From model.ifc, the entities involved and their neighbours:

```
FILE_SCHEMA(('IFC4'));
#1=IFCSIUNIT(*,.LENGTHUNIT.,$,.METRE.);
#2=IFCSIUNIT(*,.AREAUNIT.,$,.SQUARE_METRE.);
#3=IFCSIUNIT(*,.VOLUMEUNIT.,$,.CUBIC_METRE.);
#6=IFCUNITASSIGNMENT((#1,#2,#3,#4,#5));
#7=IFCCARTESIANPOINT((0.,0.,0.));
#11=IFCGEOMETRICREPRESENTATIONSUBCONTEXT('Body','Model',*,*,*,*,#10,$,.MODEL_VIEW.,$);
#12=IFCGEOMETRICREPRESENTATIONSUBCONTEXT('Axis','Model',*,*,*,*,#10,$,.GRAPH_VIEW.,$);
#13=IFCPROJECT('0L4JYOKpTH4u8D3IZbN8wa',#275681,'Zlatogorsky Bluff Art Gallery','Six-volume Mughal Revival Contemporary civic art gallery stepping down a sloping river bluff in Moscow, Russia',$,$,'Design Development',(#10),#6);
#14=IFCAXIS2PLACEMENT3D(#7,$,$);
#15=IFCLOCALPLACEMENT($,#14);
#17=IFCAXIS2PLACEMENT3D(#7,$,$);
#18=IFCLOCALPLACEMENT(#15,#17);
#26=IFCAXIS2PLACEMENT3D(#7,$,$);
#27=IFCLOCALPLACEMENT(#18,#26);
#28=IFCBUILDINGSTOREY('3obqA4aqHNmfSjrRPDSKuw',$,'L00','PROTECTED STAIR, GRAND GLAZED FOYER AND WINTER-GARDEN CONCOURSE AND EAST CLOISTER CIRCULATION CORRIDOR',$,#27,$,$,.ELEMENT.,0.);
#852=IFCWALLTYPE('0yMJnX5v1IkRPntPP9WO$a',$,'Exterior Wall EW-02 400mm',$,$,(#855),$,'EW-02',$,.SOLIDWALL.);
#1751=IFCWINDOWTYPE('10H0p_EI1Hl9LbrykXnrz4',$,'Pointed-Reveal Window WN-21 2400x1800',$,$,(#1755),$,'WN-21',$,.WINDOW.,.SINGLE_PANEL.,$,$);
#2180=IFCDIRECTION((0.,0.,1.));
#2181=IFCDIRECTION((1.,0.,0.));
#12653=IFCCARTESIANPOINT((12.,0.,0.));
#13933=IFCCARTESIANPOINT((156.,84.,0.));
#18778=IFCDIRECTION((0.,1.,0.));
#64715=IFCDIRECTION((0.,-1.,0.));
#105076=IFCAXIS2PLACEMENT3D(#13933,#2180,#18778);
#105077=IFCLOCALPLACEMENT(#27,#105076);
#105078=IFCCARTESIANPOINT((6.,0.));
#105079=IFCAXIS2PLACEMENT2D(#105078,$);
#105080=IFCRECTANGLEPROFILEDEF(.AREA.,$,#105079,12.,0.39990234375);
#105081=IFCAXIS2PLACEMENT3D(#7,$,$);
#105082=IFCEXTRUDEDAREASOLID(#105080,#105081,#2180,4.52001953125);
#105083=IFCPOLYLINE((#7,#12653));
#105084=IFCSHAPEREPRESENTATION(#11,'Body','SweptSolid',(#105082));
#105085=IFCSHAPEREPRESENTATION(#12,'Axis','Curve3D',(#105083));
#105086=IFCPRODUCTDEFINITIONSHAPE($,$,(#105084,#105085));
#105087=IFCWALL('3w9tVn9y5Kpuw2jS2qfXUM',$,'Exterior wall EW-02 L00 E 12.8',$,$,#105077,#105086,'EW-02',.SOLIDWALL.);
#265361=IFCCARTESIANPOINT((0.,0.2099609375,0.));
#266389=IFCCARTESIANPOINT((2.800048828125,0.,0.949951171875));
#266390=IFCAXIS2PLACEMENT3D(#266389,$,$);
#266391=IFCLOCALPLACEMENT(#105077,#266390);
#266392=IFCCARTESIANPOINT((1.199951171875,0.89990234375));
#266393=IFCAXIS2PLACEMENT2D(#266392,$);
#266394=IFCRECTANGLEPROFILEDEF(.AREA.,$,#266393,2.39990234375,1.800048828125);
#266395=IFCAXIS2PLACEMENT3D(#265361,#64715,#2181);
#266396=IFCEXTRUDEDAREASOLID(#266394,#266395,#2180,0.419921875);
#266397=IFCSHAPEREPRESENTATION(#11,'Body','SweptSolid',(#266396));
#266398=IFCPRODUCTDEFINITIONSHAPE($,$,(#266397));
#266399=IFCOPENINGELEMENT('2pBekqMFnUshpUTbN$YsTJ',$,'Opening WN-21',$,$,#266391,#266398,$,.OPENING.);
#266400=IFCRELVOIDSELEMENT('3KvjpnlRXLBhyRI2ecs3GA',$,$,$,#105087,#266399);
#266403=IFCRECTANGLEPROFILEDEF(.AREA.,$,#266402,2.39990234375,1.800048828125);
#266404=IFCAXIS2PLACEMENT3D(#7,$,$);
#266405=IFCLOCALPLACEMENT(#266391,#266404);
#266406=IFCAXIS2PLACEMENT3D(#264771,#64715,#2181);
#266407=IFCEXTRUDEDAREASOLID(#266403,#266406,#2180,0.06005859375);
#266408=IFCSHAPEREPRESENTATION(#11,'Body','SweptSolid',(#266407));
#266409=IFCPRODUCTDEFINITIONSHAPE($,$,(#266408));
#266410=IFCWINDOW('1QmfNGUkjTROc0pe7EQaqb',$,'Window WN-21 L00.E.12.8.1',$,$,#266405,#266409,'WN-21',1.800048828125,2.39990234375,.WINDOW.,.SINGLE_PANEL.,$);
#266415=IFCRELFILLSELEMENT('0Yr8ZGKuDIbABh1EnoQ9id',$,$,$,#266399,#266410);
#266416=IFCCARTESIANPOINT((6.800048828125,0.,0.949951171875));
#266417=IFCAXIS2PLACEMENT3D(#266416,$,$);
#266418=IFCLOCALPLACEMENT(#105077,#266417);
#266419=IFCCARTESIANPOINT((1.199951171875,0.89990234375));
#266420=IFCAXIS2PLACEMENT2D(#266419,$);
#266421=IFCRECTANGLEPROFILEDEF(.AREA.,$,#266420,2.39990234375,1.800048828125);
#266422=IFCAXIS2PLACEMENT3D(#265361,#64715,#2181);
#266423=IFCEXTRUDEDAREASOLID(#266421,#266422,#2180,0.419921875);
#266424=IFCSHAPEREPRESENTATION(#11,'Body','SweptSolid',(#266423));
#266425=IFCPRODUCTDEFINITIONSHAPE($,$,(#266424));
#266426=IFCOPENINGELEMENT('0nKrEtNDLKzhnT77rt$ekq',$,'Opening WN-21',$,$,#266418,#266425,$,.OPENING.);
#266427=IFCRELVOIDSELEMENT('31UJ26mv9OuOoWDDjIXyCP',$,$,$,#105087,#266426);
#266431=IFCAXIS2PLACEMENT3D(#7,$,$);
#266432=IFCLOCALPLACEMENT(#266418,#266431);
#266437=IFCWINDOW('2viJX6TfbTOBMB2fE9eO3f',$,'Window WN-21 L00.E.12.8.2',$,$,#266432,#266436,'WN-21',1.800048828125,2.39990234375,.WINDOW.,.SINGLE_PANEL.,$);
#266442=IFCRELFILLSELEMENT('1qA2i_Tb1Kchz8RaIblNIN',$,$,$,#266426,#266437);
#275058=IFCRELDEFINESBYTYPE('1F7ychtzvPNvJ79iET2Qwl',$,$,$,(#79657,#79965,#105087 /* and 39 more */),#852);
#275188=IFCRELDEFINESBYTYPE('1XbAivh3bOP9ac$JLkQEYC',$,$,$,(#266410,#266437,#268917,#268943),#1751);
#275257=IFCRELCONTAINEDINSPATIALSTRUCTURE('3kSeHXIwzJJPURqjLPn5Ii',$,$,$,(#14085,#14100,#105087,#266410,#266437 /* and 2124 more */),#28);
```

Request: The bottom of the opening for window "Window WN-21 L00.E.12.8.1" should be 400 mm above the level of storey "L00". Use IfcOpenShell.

```python
import numpy as np
import ifcopenshell
import ifcopenshell.api.geometry
import ifcopenshell.geom
import ifcopenshell.util.element
import ifcopenshell.util.placement
import ifcopenshell.util.shape
import ifcopenshell.util.unit

model = ifcopenshell.open("model.ifc")
unit_scale = ifcopenshell.util.unit.calculate_unit_scale(model)

window = model.by_id(266410)
opening = window.FillsVoids[0].RelatingOpeningElement
storey = ifcopenshell.util.element.get_container(window, ifc_class="IfcBuildingStorey")
level = ifcopenshell.util.placement.get_local_placement(storey.ObjectPlacement)[2, 3]

# The opening's origin need not be at the sill, so measure its lowest point.
shape = ifcopenshell.geom.create_shape(ifcopenshell.geom.settings(), opening)
bottom = ifcopenshell.util.shape.get_shape_bottom_elevation(shape, shape.geometry) / unit_scale
dz = level + 0.4 / unit_scale - bottom

shift = np.array([0.0, 0.0, dz])
# The window is placed relative to its opening, so it follows when the opening moves.
matrix = ifcopenshell.util.placement.get_local_placement(opening.ObjectPlacement)
matrix[:3, 3] += shift
ifcopenshell.api.geometry.edit_object_placement(
    model, product=opening, matrix=matrix, is_si=False, should_transform_children=True
)

print(f"moved by {dz * unit_scale:+.3f} m")

model.write("model_rev.ifc")
```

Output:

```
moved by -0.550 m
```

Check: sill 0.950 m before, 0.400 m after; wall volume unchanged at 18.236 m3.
